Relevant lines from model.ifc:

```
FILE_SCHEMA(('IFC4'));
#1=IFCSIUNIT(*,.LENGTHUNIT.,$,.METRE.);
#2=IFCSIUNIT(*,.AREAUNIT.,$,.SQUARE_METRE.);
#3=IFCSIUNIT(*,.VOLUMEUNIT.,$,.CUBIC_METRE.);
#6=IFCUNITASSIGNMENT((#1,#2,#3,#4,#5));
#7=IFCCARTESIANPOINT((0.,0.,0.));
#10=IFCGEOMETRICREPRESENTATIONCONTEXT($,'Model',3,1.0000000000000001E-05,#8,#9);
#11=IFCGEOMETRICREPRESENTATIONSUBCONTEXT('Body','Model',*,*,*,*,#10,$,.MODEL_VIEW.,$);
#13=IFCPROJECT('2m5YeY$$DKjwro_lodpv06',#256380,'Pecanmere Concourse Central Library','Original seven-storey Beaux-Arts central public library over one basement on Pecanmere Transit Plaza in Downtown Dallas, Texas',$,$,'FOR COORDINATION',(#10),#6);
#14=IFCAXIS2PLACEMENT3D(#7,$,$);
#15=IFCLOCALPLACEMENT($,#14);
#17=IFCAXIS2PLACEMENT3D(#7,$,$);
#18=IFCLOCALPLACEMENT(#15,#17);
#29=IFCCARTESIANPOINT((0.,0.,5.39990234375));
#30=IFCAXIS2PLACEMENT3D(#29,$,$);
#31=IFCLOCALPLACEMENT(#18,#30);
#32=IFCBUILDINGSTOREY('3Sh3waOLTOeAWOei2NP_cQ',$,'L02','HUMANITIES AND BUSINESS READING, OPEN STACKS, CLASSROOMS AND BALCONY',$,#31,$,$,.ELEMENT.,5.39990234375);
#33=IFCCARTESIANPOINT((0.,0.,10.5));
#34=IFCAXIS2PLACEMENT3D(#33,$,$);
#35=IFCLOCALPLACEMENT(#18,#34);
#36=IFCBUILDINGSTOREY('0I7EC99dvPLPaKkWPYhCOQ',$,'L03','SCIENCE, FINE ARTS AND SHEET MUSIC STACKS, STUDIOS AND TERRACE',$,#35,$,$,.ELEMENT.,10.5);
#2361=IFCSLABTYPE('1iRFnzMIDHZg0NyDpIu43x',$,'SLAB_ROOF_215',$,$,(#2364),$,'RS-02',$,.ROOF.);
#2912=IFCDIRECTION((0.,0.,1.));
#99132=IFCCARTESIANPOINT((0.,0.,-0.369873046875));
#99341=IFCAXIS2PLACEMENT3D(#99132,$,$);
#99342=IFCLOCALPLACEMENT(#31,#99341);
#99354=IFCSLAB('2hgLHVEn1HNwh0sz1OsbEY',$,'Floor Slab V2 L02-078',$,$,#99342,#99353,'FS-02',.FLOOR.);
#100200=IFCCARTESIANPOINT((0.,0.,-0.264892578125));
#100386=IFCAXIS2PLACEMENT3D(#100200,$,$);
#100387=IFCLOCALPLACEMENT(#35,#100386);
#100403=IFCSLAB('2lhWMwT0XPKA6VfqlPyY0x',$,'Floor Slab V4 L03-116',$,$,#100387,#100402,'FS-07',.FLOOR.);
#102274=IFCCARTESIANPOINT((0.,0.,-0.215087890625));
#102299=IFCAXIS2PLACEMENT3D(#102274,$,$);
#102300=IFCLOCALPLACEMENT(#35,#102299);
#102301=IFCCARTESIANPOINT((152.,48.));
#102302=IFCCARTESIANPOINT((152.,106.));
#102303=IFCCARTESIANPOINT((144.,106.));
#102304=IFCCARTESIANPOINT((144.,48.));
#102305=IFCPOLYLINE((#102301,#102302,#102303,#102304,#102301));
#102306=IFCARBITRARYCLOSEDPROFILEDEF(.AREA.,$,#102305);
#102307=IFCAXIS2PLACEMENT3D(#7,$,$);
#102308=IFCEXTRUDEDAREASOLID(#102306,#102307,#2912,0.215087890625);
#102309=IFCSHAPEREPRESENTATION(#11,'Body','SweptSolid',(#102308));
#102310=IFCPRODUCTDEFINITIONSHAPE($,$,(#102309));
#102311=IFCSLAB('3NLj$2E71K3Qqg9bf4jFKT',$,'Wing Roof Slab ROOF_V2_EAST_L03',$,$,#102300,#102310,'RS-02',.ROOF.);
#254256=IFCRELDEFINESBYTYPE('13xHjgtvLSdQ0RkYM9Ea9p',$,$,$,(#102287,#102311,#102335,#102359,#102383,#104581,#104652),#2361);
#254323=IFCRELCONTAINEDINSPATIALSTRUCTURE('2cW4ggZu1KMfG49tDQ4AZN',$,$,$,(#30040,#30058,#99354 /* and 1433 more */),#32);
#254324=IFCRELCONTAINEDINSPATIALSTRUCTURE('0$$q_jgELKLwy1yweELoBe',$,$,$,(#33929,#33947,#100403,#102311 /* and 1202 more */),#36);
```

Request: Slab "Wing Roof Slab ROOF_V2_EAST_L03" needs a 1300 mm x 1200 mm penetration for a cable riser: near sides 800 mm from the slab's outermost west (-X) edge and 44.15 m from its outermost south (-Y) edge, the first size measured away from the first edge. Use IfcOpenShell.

```python
import numpy as np
import ifcopenshell
import ifcopenshell.api.feature
import ifcopenshell.api.geometry
import ifcopenshell.api.root
import ifcopenshell.geom
import ifcopenshell.util.placement
import ifcopenshell.util.representation
import ifcopenshell.util.shape
import ifcopenshell.util.unit

model = ifcopenshell.open("model.ifc")
unit_scale = ifcopenshell.util.unit.calculate_unit_scale(model)
settings = ifcopenshell.geom.settings()


def volume(element):
    """Net volume in cubic metres, openings subtracted."""
    shape = ifcopenshell.geom.create_shape(settings, element)
    return ifcopenshell.util.shape.get_volume(shape.geometry)


slab = model.by_id(102311)
before = volume(slab)

# Extent in the slab's own axes, in metres. The edges named are its -X and -Y sides.
slab_shape = ifcopenshell.geom.create_shape(settings, slab)
vertices = ifcopenshell.util.shape.get_vertices(slab_shape.geometry)
x_min, y_min, bottom = vertices.min(axis=0)
top = vertices[:, 2].max()

opening = ifcopenshell.api.root.create_entity(model, ifc_class="IfcOpeningElement", name="Cable riser opening", predefined_type="OPENING")
context = ifcopenshell.util.representation.get_context(model, "Model", "Body", "MODEL_VIEW")
width, depth = 1.3, 1.2
outline = [(0.0, 0.0), (width, 0.0), (width, depth), (0.0, depth), (0.0, 0.0)]
# Overshoot both faces by 50 mm so the cut is clean.
shape = ifcopenshell.api.geometry.add_slab_representation(
    model, context=context, depth=top - bottom + 0.1, polyline=outline
)
ifcopenshell.api.geometry.assign_representation(model, product=opening, representation=shape)

matrix = ifcopenshell.util.placement.get_local_placement(slab.ObjectPlacement)
matrix[:, 3] = matrix @ np.append(np.array([x_min + 0.8, y_min + 44.15, bottom - 0.05]) / unit_scale, 1.0)
ifcopenshell.api.geometry.edit_object_placement(model, product=opening, matrix=matrix, is_si=False)
ifcopenshell.api.feature.add_feature(model, feature=opening, element=slab)

after = volume(slab)

print(f"slab volume {before:.3f} -> {after:.3f} m3")

model.write("model_updated.ifc")
```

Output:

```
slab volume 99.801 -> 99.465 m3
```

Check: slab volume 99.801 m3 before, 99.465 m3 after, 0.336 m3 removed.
